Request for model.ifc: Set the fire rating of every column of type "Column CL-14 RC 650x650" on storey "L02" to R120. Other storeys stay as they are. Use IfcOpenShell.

First a look at what the model holds.

```python
import ifcopenshell
import ifcopenshell.util.element

model = ifcopenshell.open("model.ifc")
print(model.schema)
storey = next(s for s in model.by_type("IfcBuildingStorey") if s.Name == "L02")
columns = [e for e in ifcopenshell.util.element.get_decomposition(storey) if e.is_a("IfcColumn")]
seen = {}
for e in columns:
    element_type = ifcopenshell.util.element.get_type(e)
    key = (element_type.Name if element_type != e and element_type else None, ifcopenshell.util.element.get_pset(e, "Pset_ColumnCommon", "FireRating"))
    seen[key] = seen.get(key, 0) + 1
for (name, value), count in sorted(seen.items(), key=str):
    print(count, "x", name, "|", value)
```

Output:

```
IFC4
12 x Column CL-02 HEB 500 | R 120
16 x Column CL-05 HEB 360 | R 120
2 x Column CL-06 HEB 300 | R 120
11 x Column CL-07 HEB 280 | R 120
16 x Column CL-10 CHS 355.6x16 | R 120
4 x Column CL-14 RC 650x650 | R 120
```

```python
import ifcopenshell
import ifcopenshell.api.pset
import ifcopenshell.util.element

model = ifcopenshell.open("model.ifc")

storey = next(s for s in model.by_type("IfcBuildingStorey") if s.Name == "L02")
columns = [e for e in ifcopenshell.util.element.get_decomposition(storey) if e.is_a("IfcColumn")]

count = 0
for e in columns:
    element_type = ifcopenshell.util.element.get_type(e)
    if element_type in (None, e) or element_type.Name != "Column CL-14 RC 650x650":
        continue
    # add_pset returns the element's existing set when there is one.
    pset = ifcopenshell.api.pset.add_pset(model, product=e, name="Pset_ColumnCommon")
    ifcopenshell.api.pset.edit_pset(model, pset=pset, properties={"FireRating": "R120"})
    count += 1

print(count, "columns updated")

model.write("model_edited.ifc")
```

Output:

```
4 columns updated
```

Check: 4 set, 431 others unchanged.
